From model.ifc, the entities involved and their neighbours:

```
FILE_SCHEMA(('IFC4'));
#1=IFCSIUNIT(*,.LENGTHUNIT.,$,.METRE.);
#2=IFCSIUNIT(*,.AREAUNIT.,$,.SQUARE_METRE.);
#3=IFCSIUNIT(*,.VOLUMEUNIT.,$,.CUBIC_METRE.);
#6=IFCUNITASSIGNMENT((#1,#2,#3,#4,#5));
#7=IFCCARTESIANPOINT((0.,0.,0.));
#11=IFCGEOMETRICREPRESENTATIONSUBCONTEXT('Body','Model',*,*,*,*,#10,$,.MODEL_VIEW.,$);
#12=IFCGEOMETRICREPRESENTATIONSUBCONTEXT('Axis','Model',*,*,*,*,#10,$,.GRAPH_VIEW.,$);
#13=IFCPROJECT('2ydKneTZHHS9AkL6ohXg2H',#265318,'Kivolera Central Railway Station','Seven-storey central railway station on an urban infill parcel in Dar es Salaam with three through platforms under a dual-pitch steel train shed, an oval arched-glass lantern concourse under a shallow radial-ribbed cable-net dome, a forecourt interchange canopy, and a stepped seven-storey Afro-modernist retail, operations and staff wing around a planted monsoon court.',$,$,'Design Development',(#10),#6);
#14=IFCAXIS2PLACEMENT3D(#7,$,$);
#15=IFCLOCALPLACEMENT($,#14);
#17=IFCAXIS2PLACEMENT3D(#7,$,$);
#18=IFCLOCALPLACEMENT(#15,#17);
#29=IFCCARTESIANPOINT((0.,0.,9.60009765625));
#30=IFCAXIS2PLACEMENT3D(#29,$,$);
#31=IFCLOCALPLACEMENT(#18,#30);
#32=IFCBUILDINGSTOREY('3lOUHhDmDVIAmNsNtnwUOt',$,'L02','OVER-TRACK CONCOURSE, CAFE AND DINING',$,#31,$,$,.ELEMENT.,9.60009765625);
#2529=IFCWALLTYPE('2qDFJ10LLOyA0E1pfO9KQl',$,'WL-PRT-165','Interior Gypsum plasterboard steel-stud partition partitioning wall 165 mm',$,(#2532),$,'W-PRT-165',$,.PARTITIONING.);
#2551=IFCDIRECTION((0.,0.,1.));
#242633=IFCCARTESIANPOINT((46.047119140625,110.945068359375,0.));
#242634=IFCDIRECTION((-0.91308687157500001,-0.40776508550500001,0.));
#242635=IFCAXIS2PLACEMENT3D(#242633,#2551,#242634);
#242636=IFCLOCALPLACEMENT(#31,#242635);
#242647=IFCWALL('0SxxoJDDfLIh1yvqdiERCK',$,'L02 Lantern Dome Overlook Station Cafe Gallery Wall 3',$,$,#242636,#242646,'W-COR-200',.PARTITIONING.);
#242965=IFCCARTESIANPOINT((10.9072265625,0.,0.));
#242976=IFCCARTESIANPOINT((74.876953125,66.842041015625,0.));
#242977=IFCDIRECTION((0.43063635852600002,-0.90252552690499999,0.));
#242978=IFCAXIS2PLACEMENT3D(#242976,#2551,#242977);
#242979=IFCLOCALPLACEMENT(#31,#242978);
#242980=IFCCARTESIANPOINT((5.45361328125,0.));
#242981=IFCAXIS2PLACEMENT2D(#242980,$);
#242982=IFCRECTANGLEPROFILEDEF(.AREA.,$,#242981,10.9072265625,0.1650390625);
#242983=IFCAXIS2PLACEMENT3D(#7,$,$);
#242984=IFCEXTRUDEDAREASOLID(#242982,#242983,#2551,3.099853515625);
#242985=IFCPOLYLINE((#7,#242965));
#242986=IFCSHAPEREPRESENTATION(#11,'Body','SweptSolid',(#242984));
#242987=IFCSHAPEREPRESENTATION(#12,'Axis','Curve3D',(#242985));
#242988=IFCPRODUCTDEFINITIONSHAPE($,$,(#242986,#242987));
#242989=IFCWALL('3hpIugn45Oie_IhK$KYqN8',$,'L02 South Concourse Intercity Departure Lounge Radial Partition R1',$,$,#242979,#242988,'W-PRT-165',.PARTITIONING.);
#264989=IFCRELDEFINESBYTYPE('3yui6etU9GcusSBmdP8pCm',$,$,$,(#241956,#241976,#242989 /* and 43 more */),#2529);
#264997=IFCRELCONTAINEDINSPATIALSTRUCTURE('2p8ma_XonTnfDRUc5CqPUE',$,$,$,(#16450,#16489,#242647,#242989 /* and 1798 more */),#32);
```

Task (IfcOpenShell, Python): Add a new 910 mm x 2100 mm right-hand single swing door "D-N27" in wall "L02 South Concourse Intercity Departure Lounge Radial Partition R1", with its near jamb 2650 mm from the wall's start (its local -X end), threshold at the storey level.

```python
import numpy as np
import ifcopenshell
import ifcopenshell.api.feature
import ifcopenshell.api.geometry
import ifcopenshell.api.root
import ifcopenshell.api.spatial
import ifcopenshell.geom
import ifcopenshell.util.element
import ifcopenshell.util.placement
import ifcopenshell.util.representation
import ifcopenshell.util.shape
import ifcopenshell.util.unit

model = ifcopenshell.open("model.ifc")
unit_scale = ifcopenshell.util.unit.calculate_unit_scale(model)
settings = ifcopenshell.geom.settings()


def volume(element):
    """Net volume in cubic metres, openings subtracted."""
    shape = ifcopenshell.geom.create_shape(settings, element)
    return ifcopenshell.util.shape.get_volume(shape.geometry)


wall = model.by_id(242989)
storey = ifcopenshell.util.element.get_container(wall, ifc_class="IfcBuildingStorey")
context = ifcopenshell.util.representation.get_context(model, "Model", "Body", "MODEL_VIEW")
before = volume(wall)

width, height, from_end, sill = 0.91, 2.1, 2.65, 0.0  # metres

# The wall runs along its own X axis, and the end named is its -X end.
wall_shape = ifcopenshell.geom.create_shape(settings, wall)
x, y, z = ifcopenshell.util.shape.get_vertices(wall_shape.geometry).T
start = x.min() + from_end
face, thickness = float(y.min()), float(y.max() - y.min())
wall_matrix = ifcopenshell.util.placement.get_local_placement(wall.ObjectPlacement)
level = ifcopenshell.util.placement.get_local_placement(storey.ObjectPlacement)[2, 3]


def in_wall(x, y):
    """Placement at x, y metres in the wall's axes, at sill height."""
    matrix = wall_matrix.copy()
    matrix[:, 3] = wall_matrix @ np.array([x / unit_scale, y / unit_scale, 0.0, 1.0])
    matrix[2, 3] = level + sill / unit_scale
    return matrix


# Opening: a box that overshoots both wall faces by 50 mm.
opening = ifcopenshell.api.root.create_entity(model, ifc_class="IfcOpeningElement", predefined_type="OPENING")
box = ifcopenshell.api.geometry.add_wall_representation(
    model, context=context, length=width, height=height, thickness=thickness + 0.1
)
ifcopenshell.api.geometry.assign_representation(model, product=opening, representation=box)
ifcopenshell.api.geometry.edit_object_placement(model, product=opening, matrix=in_wall(start, face - 0.05), is_si=False)
ifcopenshell.api.feature.add_feature(model, feature=opening, element=wall)

door = ifcopenshell.api.root.create_entity(model, ifc_class="IfcDoor", name="D-N27", predefined_type="DOOR")
door.OverallWidth, door.OverallHeight = width / unit_scale, height / unit_scale
door.OperationType = "SINGLE_SWING_RIGHT"
body = ifcopenshell.api.geometry.add_door_representation(
    model,
    context=context,
    overall_width=door.OverallWidth,
    overall_height=door.OverallHeight,
    operation_type="SINGLE_SWING_RIGHT",
    lining_properties={"LiningDepth": thickness / unit_scale, "ThresholdDepth": thickness / unit_scale},
)
ifcopenshell.api.geometry.assign_representation(model, product=door, representation=body)
ifcopenshell.api.spatial.assign_container(model, products=[door], relating_structure=storey)
ifcopenshell.api.feature.add_filling(model, opening=opening, element=door)

# The lining spans the wall, so the door starts at the wall face.
ifcopenshell.api.geometry.edit_object_placement(model, product=door, matrix=in_wall(start, face), is_si=False)

after = volume(wall)

print(f"wall volume {before:.3f} -> {after:.3f} m3")

model.write("model-out.ifc")
```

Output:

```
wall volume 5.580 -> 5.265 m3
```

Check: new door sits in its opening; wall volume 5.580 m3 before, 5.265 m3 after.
